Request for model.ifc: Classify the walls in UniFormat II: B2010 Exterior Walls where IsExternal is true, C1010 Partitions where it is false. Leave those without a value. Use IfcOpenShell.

First a look at what the model holds.

```python
import ifcopenshell
import ifcopenshell.util.element

model = ifcopenshell.open("model.ifc")
print(model.schema)
print("classifications:", [c.Name for c in model.by_type("IfcClassification")])
values = [ifcopenshell.util.element.get_pset(e, "Pset_WallCommon", "IsExternal") for e in model.by_type("IfcWall")]
for value in (True, False, None):
    print("IsExternal", value, values.count(value))
```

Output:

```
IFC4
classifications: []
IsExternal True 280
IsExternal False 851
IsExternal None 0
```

```python
import ifcopenshell
import ifcopenshell.api.classification
import ifcopenshell.util.element

model = ifcopenshell.open("model.ifc")

system = ifcopenshell.api.classification.add_classification(model, classification="UniFormat II")

walls = model.by_type("IfcWall")
external = {e: ifcopenshell.util.element.get_pset(e, "Pset_WallCommon", "IsExternal") for e in walls}
for flag, code, name in ((True, "B2010", "Exterior Walls"), (False, "C1010", "Partitions")):
    products = [e for e in walls if external[e] is flag]
    ifcopenshell.api.classification.add_reference(
        model, products=products, classification=system, identification=code, name=name
    )
    print(code, len(products))

model.write("model_v2.ifc")
```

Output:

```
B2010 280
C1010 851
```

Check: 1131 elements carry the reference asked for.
